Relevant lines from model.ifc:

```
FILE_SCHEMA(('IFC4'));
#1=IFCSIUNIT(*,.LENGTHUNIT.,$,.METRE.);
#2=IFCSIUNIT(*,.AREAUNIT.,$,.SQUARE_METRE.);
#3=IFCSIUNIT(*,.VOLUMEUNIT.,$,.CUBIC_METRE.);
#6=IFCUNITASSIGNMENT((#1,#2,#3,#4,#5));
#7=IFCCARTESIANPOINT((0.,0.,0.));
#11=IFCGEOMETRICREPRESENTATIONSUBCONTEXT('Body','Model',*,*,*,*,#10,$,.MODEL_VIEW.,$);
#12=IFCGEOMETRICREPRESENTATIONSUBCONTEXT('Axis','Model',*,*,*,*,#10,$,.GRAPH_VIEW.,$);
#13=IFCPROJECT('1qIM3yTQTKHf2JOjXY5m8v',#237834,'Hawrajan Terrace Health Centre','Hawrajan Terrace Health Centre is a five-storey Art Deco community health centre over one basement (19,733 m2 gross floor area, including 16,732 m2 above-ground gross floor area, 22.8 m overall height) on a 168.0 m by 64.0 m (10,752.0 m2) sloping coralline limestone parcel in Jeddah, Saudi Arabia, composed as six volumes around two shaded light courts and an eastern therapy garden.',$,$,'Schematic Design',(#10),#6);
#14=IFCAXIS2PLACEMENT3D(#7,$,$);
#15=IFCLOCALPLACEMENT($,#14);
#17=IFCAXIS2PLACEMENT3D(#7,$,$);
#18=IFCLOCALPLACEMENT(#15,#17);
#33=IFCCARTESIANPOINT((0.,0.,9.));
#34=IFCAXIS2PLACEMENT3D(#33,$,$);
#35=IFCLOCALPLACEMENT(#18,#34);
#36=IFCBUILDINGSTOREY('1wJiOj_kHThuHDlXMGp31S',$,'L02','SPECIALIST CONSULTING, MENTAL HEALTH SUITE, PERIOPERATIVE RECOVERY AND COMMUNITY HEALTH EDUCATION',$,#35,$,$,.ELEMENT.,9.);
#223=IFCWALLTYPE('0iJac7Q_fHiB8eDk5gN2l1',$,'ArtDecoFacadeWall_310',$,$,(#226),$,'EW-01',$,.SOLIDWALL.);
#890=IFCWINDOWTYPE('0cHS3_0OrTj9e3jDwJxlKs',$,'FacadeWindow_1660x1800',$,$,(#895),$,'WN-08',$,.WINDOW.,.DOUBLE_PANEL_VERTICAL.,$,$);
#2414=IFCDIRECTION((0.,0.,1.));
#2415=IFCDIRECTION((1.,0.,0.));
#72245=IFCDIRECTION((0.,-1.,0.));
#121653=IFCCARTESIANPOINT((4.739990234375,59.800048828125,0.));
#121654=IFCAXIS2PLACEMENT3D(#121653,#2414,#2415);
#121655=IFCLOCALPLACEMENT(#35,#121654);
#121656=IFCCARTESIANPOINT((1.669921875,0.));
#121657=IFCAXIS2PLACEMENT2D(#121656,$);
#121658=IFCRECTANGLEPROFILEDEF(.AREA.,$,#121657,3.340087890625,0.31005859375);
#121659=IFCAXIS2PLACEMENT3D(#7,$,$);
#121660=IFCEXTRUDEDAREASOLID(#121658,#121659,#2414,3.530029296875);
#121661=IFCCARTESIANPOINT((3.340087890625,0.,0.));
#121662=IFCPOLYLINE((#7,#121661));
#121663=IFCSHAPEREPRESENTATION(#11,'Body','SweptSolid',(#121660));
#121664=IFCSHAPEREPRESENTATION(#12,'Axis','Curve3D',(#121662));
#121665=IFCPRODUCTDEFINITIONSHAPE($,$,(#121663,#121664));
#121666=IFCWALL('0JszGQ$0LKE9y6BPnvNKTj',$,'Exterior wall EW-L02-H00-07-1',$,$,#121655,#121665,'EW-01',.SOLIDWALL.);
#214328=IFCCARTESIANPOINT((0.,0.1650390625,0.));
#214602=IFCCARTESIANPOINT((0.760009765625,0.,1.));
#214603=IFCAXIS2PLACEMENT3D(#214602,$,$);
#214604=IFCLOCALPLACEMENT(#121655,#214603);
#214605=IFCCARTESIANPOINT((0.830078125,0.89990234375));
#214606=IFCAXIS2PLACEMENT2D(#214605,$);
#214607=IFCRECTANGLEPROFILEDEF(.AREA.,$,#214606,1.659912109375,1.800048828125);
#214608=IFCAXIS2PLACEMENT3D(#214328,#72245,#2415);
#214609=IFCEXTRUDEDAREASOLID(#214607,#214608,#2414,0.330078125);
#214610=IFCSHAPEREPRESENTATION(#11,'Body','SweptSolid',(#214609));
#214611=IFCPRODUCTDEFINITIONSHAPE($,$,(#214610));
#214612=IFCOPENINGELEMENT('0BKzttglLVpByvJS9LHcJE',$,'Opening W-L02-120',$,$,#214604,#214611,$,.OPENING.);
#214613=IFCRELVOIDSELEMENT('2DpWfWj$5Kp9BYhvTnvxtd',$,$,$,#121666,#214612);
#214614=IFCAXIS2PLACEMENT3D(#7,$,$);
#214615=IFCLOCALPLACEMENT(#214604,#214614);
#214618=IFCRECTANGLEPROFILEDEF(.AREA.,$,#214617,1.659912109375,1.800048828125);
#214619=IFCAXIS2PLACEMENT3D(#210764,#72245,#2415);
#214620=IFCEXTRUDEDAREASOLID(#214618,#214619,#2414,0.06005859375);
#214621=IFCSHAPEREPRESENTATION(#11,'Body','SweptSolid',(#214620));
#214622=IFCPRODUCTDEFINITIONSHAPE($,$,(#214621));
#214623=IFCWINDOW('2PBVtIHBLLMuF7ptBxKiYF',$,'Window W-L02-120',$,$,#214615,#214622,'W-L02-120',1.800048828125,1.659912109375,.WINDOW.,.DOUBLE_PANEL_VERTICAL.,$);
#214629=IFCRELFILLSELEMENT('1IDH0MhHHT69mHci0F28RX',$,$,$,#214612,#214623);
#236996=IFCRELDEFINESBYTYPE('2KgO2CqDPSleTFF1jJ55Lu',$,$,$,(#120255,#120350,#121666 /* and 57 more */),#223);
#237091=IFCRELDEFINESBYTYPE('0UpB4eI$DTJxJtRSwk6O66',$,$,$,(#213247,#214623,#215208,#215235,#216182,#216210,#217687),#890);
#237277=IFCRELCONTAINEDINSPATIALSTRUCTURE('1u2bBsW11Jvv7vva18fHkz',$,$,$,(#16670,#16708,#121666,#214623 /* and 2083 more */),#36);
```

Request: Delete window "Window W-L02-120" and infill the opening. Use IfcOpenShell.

```python
import ifcopenshell
import ifcopenshell.api.feature
import ifcopenshell.api.root
import ifcopenshell.geom
import ifcopenshell.util.shape

model = ifcopenshell.open("model.ifc")
settings = ifcopenshell.geom.settings()


def volume(element):
    """Net volume in cubic metres, openings subtracted."""
    shape = ifcopenshell.geom.create_shape(settings, element)
    return ifcopenshell.util.shape.get_volume(shape.geometry)


window = model.by_guid("2PBVtIHBLLMuF7ptBxKiYF")
opening = window.FillsVoids[0].RelatingOpeningElement
wall = opening.VoidsElements[0].RelatingBuildingElement
before = volume(wall)

ifcopenshell.api.root.remove_product(model, product=window)
ifcopenshell.api.feature.remove_feature(model, feature=opening)

after = volume(wall)

print(f"wall volume {before:.3f} -> {after:.3f} m3")

model.write("model_v2.ifc")
```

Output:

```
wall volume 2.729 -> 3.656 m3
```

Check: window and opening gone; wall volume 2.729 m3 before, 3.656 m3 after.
